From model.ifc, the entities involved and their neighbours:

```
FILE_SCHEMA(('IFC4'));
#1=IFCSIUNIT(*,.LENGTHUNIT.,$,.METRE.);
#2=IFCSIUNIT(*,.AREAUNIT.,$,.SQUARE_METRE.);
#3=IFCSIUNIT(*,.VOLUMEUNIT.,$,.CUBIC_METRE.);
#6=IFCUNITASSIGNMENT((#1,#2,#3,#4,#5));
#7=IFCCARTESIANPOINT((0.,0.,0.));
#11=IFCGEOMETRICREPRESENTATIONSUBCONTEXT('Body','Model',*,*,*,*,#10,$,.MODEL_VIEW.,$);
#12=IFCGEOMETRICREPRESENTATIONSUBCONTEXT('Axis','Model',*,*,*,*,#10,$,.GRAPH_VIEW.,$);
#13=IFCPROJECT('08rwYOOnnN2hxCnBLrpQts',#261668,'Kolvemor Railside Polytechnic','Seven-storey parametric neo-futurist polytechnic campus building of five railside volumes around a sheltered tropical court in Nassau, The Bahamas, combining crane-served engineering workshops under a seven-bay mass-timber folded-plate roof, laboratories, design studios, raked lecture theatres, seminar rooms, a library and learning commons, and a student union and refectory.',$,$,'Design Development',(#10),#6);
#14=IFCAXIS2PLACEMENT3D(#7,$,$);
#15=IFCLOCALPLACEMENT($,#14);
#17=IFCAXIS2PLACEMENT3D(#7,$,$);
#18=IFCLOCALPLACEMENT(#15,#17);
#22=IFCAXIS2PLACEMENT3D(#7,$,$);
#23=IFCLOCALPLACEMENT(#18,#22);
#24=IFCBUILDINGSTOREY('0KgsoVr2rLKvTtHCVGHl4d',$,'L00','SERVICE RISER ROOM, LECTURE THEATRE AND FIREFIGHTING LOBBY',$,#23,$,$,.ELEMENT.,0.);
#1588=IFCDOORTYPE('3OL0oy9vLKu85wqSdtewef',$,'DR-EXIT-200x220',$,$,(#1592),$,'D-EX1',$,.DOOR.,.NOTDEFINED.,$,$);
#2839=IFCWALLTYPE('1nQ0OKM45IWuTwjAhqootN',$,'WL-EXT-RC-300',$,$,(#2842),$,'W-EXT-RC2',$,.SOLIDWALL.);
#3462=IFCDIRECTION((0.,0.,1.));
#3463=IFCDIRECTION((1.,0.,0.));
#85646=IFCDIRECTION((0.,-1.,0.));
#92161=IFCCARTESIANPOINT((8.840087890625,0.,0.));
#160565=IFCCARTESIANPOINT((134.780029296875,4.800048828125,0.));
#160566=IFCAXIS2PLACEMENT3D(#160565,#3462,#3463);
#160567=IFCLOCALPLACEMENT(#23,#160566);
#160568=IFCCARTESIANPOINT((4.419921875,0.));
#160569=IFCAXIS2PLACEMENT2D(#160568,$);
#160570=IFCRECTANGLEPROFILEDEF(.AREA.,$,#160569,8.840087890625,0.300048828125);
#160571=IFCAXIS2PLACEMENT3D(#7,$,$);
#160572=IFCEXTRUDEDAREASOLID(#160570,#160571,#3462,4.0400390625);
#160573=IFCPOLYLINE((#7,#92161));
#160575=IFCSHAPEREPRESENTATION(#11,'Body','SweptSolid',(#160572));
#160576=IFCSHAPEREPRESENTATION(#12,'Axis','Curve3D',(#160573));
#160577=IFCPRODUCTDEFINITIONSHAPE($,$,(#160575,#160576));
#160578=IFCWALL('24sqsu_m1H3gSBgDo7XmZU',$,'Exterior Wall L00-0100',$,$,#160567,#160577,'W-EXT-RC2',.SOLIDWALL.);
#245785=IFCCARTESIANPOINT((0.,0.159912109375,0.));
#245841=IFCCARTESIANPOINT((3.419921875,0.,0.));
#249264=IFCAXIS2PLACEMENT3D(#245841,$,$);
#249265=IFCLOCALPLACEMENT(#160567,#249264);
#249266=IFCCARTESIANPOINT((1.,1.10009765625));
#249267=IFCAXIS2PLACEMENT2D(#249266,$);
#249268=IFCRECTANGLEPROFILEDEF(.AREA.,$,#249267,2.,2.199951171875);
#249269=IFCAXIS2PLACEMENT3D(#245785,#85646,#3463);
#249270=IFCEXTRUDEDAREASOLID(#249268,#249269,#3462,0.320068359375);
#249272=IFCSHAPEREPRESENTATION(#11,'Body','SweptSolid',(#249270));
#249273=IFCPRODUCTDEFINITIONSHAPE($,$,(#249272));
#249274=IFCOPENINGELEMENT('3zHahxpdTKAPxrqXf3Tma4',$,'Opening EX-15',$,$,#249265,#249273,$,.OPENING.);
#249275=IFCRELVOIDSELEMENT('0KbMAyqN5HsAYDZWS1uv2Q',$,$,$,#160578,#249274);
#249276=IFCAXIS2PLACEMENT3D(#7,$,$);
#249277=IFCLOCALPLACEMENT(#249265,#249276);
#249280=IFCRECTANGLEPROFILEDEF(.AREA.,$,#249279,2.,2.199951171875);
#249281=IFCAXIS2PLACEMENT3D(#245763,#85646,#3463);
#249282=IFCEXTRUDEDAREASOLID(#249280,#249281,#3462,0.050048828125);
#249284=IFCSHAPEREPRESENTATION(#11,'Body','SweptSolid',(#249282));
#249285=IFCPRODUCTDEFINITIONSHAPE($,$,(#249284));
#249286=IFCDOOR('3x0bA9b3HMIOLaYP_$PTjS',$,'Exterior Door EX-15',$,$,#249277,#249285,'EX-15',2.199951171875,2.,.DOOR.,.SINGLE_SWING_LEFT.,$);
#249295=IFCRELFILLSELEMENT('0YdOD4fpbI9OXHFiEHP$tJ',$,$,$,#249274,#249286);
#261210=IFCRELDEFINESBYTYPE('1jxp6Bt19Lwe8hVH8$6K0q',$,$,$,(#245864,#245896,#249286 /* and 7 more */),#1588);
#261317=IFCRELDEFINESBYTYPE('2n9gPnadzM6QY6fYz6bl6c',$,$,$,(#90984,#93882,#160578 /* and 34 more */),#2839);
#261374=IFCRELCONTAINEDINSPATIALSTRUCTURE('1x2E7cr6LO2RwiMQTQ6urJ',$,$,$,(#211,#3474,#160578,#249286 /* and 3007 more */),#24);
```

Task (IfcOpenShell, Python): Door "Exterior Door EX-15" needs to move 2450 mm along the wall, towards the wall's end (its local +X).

```python
import ifcopenshell
import ifcopenshell.api.geometry
import ifcopenshell.util.placement

model = ifcopenshell.open("model.ifc")

door = model.by_guid("3x0bA9b3HMIOLaYP_$PTjS")
opening = door.FillsVoids[0].RelatingOpeningElement
wall = opening.VoidsElements[0].RelatingBuildingElement

wall_matrix = ifcopenshell.util.placement.get_local_placement(wall.ObjectPlacement)
shift = wall_matrix[:3, 0] * 2.45
before = ifcopenshell.util.placement.get_local_placement(door.ObjectPlacement)[:3, 3].copy()

# The door is placed relative to its opening, so it follows when the opening moves.
matrix = ifcopenshell.util.placement.get_local_placement(opening.ObjectPlacement)
matrix[:3, 3] += shift
ifcopenshell.api.geometry.edit_object_placement(
    model, product=opening, matrix=matrix, is_si=False, should_transform_children=True
)

after = ifcopenshell.util.placement.get_local_placement(door.ObjectPlacement)[:3, 3]
print("door moved by", (after - before).round(3) + 0.0)

model.write("model_edited.ifc")
```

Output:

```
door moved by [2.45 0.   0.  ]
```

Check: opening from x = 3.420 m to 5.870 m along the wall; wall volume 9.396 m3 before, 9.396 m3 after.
